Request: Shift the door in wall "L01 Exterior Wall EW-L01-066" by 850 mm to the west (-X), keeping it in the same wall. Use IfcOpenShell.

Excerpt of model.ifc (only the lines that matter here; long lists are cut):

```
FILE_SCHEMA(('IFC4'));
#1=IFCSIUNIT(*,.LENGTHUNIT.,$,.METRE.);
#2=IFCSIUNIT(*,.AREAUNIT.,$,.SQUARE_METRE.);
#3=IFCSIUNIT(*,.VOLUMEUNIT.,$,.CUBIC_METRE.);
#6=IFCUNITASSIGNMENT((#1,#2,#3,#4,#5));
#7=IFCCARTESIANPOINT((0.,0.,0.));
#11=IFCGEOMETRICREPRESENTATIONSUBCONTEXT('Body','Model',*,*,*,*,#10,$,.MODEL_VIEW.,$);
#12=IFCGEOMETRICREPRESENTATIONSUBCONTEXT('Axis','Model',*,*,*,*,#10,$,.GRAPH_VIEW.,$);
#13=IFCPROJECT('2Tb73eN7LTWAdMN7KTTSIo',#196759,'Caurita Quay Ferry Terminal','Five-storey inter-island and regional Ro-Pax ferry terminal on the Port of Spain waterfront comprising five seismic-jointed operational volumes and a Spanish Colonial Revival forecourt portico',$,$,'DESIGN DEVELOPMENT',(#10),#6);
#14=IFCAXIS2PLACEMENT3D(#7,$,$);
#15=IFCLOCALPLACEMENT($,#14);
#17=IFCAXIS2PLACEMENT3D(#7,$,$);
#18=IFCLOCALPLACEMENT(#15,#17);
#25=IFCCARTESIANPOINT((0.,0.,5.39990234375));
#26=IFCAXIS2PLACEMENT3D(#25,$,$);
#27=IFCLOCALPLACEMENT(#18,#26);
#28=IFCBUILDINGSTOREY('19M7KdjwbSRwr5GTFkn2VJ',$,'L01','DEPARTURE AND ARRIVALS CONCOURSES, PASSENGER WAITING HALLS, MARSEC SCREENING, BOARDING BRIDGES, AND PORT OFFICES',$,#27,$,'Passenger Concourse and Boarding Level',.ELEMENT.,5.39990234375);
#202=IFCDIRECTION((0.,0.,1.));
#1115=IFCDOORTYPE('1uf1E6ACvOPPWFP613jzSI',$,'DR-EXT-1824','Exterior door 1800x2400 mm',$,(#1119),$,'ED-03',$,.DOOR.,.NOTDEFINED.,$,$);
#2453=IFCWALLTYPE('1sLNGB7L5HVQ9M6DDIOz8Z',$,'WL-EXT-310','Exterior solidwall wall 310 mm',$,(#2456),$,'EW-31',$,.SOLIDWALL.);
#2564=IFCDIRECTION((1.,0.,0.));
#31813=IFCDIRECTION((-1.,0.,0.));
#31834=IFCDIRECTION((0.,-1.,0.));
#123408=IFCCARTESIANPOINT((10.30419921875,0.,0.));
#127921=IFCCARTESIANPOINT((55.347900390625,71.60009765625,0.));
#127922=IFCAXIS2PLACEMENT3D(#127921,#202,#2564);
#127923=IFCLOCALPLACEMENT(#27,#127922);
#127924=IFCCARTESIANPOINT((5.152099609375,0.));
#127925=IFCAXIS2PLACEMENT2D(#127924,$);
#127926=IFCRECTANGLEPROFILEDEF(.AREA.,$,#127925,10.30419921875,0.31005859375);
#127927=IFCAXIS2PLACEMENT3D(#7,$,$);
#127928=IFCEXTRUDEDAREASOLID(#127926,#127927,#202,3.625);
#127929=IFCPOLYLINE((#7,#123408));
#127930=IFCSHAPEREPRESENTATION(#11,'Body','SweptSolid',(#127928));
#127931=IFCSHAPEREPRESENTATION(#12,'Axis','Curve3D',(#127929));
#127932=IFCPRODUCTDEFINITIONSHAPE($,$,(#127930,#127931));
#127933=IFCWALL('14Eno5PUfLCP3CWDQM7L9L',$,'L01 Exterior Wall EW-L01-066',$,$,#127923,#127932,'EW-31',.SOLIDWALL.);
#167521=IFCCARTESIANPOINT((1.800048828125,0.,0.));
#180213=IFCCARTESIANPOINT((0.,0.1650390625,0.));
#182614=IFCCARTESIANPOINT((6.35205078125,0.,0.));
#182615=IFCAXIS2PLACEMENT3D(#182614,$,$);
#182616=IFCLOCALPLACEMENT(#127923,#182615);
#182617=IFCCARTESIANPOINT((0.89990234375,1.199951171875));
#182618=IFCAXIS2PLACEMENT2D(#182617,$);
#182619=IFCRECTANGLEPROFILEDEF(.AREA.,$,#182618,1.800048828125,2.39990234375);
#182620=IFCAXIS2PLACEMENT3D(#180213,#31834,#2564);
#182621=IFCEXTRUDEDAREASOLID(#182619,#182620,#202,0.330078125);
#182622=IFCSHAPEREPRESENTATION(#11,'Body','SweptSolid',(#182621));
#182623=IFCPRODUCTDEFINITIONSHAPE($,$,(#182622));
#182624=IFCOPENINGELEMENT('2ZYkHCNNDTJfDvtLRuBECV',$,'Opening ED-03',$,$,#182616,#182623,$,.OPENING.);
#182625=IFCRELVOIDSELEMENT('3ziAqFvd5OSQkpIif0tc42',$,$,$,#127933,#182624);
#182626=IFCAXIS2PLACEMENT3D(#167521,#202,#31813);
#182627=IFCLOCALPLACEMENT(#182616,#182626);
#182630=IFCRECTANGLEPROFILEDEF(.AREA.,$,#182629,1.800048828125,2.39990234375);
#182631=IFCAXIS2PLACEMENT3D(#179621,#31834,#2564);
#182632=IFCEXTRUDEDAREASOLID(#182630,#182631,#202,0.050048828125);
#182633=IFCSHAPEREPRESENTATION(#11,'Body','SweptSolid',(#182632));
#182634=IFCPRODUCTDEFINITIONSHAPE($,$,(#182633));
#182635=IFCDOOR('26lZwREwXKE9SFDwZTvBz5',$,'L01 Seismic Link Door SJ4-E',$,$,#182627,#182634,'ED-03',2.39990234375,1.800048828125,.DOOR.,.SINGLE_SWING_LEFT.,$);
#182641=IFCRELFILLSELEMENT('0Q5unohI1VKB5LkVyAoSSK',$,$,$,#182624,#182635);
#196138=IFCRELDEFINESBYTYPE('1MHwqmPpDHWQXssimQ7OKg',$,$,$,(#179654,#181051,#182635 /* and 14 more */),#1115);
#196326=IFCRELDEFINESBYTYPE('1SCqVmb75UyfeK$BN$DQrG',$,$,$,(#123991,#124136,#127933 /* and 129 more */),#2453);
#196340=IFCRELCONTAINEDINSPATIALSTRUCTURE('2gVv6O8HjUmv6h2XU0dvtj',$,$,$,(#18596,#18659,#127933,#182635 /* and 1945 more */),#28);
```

```python
import ifcopenshell
import ifcopenshell.api.geometry
import ifcopenshell.util.placement
import ifcopenshell.util.unit

model = ifcopenshell.open("model.ifc")
unit_scale = ifcopenshell.util.unit.calculate_unit_scale(model)

door = model.by_guid("26lZwREwXKE9SFDwZTvBz5")
opening = door.FillsVoids[0].RelatingOpeningElement
wall = opening.VoidsElements[0].RelatingBuildingElement

wall_matrix = ifcopenshell.util.placement.get_local_placement(wall.ObjectPlacement)
shift = wall_matrix[:3, 0] * -0.85 / unit_scale
before = ifcopenshell.util.placement.get_local_placement(door.ObjectPlacement)[:3, 3].copy()

# The door is placed relative to its opening, so it follows when the opening moves.
matrix = ifcopenshell.util.placement.get_local_placement(opening.ObjectPlacement)
matrix[:3, 3] += shift
ifcopenshell.api.geometry.edit_object_placement(
    model, product=opening, matrix=matrix, is_si=False, should_transform_children=True
)

after = ifcopenshell.util.placement.get_local_placement(door.ObjectPlacement)[:3, 3]
print("door moved by", (after - before).round(3) + 0.0)

model.write("model_rev.ifc")
```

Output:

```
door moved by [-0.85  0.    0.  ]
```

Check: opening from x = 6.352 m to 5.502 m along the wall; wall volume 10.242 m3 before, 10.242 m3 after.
